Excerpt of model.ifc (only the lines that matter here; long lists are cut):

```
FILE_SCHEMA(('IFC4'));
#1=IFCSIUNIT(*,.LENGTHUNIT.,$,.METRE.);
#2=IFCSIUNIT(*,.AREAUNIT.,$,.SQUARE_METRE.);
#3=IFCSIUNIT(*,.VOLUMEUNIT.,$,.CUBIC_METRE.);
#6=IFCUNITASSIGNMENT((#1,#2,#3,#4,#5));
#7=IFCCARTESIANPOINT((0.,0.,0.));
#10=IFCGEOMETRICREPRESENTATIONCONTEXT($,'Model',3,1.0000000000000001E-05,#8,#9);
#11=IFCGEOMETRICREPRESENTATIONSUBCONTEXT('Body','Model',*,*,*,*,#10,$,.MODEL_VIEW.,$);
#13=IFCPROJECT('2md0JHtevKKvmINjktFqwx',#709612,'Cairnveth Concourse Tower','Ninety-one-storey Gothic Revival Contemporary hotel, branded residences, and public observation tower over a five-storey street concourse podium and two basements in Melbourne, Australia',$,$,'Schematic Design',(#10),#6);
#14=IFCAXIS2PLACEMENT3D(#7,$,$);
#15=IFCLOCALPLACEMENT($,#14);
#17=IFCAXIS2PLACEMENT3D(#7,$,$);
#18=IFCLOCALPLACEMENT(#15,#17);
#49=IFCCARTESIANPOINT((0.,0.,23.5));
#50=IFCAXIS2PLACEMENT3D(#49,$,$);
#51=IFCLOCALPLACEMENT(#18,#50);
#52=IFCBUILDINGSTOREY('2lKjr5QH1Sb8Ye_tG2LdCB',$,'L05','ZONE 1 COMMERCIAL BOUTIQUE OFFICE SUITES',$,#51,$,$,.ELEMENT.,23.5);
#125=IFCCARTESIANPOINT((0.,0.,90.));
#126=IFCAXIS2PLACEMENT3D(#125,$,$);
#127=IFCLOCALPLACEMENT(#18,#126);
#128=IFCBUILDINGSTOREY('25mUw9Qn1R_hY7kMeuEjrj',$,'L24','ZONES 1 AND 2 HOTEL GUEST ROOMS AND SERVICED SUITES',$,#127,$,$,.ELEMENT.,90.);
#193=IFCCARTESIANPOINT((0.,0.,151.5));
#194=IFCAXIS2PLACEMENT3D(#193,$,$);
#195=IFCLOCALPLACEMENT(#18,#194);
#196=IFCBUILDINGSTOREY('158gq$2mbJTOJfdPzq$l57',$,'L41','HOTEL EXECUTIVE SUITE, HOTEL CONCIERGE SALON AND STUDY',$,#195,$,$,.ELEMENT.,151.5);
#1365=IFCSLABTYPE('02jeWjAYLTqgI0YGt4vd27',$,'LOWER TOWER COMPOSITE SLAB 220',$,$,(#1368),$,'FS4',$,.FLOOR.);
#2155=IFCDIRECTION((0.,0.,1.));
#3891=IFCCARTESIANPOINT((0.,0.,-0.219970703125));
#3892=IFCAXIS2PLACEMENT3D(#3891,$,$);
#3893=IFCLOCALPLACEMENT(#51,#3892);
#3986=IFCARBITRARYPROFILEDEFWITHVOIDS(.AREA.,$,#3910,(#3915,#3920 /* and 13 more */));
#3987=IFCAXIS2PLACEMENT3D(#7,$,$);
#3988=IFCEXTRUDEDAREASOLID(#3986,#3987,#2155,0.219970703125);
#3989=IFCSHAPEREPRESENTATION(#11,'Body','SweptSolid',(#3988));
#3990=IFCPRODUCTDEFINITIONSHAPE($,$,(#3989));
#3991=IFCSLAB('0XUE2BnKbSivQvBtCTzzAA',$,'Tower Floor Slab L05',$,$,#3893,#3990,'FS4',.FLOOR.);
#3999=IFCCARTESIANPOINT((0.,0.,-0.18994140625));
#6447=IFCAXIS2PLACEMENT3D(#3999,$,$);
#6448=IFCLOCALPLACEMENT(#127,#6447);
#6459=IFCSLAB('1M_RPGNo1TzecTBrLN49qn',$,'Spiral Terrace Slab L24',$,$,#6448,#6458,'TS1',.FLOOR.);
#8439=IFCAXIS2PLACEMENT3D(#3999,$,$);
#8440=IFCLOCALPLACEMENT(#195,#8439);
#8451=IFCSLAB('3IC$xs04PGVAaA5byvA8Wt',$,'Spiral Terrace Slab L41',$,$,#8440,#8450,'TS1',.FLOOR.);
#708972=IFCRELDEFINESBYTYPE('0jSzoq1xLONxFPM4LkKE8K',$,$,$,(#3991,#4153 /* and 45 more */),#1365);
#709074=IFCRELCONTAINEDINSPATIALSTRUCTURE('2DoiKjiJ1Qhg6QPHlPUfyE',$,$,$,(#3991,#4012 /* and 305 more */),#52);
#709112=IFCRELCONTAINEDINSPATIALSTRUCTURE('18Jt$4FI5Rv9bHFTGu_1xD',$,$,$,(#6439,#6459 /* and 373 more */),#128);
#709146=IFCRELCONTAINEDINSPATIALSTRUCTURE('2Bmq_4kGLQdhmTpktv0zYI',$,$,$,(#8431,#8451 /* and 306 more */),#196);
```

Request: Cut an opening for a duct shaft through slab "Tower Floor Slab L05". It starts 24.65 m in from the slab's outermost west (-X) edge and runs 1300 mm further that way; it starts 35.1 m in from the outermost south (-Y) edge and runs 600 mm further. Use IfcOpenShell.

```python
import numpy as np
import ifcopenshell
import ifcopenshell.api.feature
import ifcopenshell.api.geometry
import ifcopenshell.api.root
import ifcopenshell.geom
import ifcopenshell.util.placement
import ifcopenshell.util.representation
import ifcopenshell.util.shape
import ifcopenshell.util.unit

model = ifcopenshell.open("model.ifc")
unit_scale = ifcopenshell.util.unit.calculate_unit_scale(model)
settings = ifcopenshell.geom.settings()


def volume(element):
    """Net volume in cubic metres, openings subtracted."""
    shape = ifcopenshell.geom.create_shape(settings, element)
    return ifcopenshell.util.shape.get_volume(shape.geometry)


slab = model.by_guid("0XUE2BnKbSivQvBtCTzzAA")
before = volume(slab)

# Extent in the slab's own axes, in metres. The edges named are its -X and -Y sides.
slab_shape = ifcopenshell.geom.create_shape(settings, slab)
vertices = ifcopenshell.util.shape.get_vertices(slab_shape.geometry)
x_min, y_min, bottom = vertices.min(axis=0)
top = vertices[:, 2].max()

opening = ifcopenshell.api.root.create_entity(model, ifc_class="IfcOpeningElement", name="Duct shaft opening", predefined_type="OPENING")
context = ifcopenshell.util.representation.get_context(model, "Model", "Body", "MODEL_VIEW")
width, depth = 1.3, 0.6
outline = [(0.0, 0.0), (width, 0.0), (width, depth), (0.0, depth), (0.0, 0.0)]
# Overshoot both faces by 50 mm so the cut is clean.
shape = ifcopenshell.api.geometry.add_slab_representation(
    model, context=context, depth=top - bottom + 0.1, polyline=outline
)
ifcopenshell.api.geometry.assign_representation(model, product=opening, representation=shape)

matrix = ifcopenshell.util.placement.get_local_placement(slab.ObjectPlacement)
matrix[:, 3] = matrix @ np.append(np.array([x_min + 24.65, y_min + 35.1, bottom - 0.05]) / unit_scale, 1.0)
ifcopenshell.api.geometry.edit_object_placement(model, product=opening, matrix=matrix, is_si=False)
ifcopenshell.api.feature.add_feature(model, feature=opening, element=slab)

after = volume(slab)

print(f"slab volume {before:.3f} -> {after:.3f} m3")

model.write("model_rev.ifc")
```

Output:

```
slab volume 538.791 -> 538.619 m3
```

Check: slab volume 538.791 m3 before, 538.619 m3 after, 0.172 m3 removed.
